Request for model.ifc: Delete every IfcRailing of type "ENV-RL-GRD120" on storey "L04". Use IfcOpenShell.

First a look at what the model holds.

```python
import ifcopenshell
import ifcopenshell.util.element

model = ifcopenshell.open("model.ifc")
print(model.schema)
storey = next(s for s in model.by_type("IfcBuildingStorey") if s.Name == "L04")
railings = [e for e in ifcopenshell.util.element.get_decomposition(storey) if e.is_a("IfcRailing")]
seen = {}
for e in railings:
    element_type = ifcopenshell.util.element.get_type(e)
    name = element_type.Name if element_type not in (None, e) else None
    seen[name] = seen.get(name, 0) + 1
for name, count in sorted(seen.items(), key=str):
    print(count, "x", name)
```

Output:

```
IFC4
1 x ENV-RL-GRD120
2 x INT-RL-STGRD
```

```python
import ifcopenshell
import ifcopenshell.api.root
import ifcopenshell.util.element

model = ifcopenshell.open("model.ifc")

storey = next(s for s in model.by_type("IfcBuildingStorey") if s.Name == "L04")
railings = [e for e in ifcopenshell.util.element.get_decomposition(storey) if e.is_a("IfcRailing")]
targets = [e for e in railings if (t := ifcopenshell.util.element.get_type(e)) not in (None, e) and t.Name == "ENV-RL-GRD120"]

for e in targets:
    ifcopenshell.api.root.remove_product(model, product=e)
print(len(targets), "removed")

model.write("model_v2.ifc")
```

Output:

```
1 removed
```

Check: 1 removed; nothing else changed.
